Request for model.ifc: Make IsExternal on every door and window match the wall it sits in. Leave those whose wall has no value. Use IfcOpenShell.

First a look at what the model holds.

```python
import ifcopenshell
import ifcopenshell.util.element

model = ifcopenshell.open("model.ifc")
print(model.schema)
seen = {}
for e in model.by_type("IfcDoor") + model.by_type("IfcWindow"):
    if not e.FillsVoids:
        continue
    host = e.FillsVoids[0].RelatingOpeningElement.VoidsElements[0].RelatingBuildingElement
    own = ifcopenshell.util.element.get_pset(e, f"Pset_{e.is_a()[3:].removesuffix('StandardCase')}Common", "IsExternal")
    wall = ifcopenshell.util.element.get_pset(host, "Pset_WallCommon", "IsExternal")
    seen[e.is_a(), own, wall] = seen.get((e.is_a(), own, wall), 0) + 1
for (cls, own, wall), count in sorted(seen.items(), key=str):
    print(count, cls, "IsExternal:", own, "| host wall:", wall)
```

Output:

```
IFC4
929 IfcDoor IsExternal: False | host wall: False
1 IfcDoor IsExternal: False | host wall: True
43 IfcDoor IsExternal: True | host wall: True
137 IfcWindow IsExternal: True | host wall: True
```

```python
import ifcopenshell
import ifcopenshell.api.pset
import ifcopenshell.util.element

model = ifcopenshell.open("model.ifc")

count = 0
for ifc_class, pset_name in (("IfcDoor", "Pset_DoorCommon"), ("IfcWindow", "Pset_WindowCommon")):
    for e in model.by_type(ifc_class):
        if not e.FillsVoids:
            continue
        host = e.FillsVoids[0].RelatingOpeningElement.VoidsElements[0].RelatingBuildingElement
        external = ifcopenshell.util.element.get_pset(host, "Pset_WallCommon", "IsExternal")
        if external is None or ifcopenshell.util.element.get_pset(e, pset_name, "IsExternal") == external:
            continue
        pset = ifcopenshell.api.pset.add_pset(model, product=e, name=pset_name)
        ifcopenshell.api.pset.edit_pset(model, pset=pset, properties={"IsExternal": external})
        count += 1

print(count, "updated")

model.write("model_rev.ifc")
```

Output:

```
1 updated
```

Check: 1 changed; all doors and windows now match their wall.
